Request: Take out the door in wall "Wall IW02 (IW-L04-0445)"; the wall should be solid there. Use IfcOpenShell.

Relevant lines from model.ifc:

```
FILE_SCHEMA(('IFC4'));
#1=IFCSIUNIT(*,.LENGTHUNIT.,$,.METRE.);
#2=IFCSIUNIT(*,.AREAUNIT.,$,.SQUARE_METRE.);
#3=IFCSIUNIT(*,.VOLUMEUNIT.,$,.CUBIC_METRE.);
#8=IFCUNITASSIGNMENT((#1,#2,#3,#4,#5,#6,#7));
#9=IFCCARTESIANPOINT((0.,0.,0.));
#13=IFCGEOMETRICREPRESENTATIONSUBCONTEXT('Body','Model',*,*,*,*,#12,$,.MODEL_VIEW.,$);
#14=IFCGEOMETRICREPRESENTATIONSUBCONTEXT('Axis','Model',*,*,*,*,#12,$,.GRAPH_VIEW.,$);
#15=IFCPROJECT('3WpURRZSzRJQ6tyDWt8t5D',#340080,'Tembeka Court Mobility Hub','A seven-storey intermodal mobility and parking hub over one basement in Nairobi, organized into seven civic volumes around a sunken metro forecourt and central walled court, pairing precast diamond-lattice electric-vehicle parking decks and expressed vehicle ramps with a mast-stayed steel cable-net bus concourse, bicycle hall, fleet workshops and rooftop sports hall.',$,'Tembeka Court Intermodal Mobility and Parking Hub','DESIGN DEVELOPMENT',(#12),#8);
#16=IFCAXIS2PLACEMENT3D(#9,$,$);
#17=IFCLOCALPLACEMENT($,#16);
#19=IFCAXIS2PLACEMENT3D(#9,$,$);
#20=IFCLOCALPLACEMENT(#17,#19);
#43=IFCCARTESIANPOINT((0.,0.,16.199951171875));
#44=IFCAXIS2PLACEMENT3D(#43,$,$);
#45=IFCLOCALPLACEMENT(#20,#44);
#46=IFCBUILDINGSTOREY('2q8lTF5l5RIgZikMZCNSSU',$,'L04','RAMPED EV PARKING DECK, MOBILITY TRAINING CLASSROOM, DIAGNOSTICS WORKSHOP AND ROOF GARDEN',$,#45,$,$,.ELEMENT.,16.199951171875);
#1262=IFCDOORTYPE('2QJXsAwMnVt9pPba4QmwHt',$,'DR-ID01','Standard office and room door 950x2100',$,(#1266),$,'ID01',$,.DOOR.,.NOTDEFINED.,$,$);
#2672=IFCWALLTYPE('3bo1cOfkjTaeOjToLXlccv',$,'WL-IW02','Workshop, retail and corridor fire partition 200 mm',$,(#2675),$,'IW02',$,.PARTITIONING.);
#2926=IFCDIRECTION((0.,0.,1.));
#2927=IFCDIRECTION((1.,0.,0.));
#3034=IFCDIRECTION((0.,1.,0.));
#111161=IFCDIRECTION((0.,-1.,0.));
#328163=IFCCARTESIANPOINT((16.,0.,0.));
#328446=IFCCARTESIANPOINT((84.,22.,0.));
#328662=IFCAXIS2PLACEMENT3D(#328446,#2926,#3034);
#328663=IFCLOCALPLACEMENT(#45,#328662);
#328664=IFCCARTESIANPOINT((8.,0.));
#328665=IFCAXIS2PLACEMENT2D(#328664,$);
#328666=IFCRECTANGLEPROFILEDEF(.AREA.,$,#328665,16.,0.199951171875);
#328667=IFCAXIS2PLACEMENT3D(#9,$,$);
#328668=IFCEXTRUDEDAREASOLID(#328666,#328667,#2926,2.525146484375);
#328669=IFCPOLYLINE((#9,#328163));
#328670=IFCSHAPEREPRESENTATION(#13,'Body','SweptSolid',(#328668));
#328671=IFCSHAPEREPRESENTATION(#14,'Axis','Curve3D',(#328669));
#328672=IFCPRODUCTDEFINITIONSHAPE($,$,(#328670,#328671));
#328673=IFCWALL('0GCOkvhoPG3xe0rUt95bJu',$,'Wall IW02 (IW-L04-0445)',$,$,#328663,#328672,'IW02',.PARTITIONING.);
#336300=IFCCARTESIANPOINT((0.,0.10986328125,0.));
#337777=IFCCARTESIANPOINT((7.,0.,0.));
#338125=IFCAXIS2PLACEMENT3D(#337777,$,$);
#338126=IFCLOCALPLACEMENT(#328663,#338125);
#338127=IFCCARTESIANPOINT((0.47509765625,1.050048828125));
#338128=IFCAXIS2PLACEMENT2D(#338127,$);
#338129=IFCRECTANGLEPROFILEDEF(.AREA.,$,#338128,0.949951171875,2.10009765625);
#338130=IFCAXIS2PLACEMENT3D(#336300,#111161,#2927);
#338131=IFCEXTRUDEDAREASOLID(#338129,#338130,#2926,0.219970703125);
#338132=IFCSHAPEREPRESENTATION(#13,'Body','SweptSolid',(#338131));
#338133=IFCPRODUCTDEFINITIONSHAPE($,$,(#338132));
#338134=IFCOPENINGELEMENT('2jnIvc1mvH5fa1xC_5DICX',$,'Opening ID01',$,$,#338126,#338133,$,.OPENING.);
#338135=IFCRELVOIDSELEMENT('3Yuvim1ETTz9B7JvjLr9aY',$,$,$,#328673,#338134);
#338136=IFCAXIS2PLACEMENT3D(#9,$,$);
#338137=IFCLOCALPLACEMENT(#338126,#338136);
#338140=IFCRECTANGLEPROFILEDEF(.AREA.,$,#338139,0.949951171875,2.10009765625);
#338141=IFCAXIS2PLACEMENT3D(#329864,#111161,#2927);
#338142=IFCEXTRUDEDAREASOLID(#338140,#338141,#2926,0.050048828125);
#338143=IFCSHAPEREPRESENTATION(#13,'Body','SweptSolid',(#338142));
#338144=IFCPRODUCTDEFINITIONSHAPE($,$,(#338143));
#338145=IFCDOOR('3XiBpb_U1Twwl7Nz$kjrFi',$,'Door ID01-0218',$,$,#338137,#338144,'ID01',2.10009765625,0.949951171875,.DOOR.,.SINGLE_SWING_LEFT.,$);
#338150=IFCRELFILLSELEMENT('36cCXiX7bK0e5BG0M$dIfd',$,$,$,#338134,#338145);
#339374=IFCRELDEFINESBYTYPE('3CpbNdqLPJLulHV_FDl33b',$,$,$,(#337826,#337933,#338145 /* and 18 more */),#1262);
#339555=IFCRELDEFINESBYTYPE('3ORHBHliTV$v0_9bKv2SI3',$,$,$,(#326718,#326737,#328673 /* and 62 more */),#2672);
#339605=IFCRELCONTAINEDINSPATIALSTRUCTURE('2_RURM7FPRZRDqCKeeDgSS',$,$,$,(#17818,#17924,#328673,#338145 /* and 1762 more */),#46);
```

```python
import ifcopenshell
import ifcopenshell.api.feature
import ifcopenshell.api.root
import ifcopenshell.geom
import ifcopenshell.util.shape

model = ifcopenshell.open("model.ifc")
settings = ifcopenshell.geom.settings()


def volume(element):
    """Net volume in cubic metres, openings subtracted."""
    shape = ifcopenshell.geom.create_shape(settings, element)
    return ifcopenshell.util.shape.get_volume(shape.geometry)


door = model.by_id(338145)
opening = door.FillsVoids[0].RelatingOpeningElement
wall = opening.VoidsElements[0].RelatingBuildingElement
before = volume(wall)

ifcopenshell.api.root.remove_product(model, product=door)
ifcopenshell.api.feature.remove_feature(model, feature=opening)

after = volume(wall)

print(f"wall volume {before:.3f} -> {after:.3f} m3")

model.write("model_rev.ifc")
```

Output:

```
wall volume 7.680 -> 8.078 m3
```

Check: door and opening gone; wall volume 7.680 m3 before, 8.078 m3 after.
